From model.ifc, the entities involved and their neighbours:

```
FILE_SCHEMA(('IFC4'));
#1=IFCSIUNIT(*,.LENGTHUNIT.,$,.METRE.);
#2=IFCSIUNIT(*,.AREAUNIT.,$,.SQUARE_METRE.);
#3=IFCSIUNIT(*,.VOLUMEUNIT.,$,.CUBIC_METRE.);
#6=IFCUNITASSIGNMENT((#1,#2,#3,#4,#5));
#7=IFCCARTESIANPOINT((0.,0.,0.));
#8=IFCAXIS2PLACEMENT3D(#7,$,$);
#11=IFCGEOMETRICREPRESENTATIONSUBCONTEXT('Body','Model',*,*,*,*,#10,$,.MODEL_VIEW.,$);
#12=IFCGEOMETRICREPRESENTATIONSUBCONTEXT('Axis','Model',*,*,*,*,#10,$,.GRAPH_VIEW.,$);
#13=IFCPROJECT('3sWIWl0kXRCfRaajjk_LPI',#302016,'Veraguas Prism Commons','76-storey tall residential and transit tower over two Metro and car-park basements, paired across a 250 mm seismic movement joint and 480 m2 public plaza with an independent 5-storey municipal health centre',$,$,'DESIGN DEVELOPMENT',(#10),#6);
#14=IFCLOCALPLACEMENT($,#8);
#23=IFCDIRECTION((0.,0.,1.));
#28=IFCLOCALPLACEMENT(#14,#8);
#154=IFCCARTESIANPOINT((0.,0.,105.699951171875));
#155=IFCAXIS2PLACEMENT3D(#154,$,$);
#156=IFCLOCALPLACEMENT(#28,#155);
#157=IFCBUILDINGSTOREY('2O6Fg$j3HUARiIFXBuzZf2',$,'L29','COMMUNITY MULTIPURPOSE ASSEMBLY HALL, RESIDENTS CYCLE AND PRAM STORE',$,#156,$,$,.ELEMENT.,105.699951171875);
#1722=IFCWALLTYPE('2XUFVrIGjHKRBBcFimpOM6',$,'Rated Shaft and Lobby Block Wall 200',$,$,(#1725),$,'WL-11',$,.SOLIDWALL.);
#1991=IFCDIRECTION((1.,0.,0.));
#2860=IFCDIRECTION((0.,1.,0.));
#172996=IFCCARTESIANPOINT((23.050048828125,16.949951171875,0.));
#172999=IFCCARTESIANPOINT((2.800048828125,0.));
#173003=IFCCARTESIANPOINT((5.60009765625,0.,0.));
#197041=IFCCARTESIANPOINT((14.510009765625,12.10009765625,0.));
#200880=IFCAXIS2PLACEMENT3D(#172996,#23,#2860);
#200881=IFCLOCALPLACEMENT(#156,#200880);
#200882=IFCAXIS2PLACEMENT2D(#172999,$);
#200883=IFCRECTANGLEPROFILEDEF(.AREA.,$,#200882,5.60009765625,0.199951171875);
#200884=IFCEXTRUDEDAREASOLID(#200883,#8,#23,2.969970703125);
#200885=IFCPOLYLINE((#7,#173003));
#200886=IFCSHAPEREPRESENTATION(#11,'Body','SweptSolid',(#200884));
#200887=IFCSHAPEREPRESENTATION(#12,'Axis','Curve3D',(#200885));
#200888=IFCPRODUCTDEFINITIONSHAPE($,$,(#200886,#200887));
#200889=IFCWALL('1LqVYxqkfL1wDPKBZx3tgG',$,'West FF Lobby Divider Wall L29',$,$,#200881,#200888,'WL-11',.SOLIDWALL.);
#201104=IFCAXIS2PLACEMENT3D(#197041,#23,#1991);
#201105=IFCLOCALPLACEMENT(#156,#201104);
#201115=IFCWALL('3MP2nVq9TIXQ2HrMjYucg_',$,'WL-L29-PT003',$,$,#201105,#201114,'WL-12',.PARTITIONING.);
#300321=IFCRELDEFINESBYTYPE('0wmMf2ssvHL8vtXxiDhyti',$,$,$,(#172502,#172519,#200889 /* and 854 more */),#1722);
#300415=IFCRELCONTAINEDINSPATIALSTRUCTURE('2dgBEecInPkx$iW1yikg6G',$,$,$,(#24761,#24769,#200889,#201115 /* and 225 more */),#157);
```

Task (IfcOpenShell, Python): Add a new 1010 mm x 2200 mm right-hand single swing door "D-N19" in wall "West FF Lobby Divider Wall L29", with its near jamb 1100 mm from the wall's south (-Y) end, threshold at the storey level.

```python
import numpy as np
import ifcopenshell
import ifcopenshell.api.feature
import ifcopenshell.api.geometry
import ifcopenshell.api.root
import ifcopenshell.api.spatial
import ifcopenshell.geom
import ifcopenshell.util.element
import ifcopenshell.util.placement
import ifcopenshell.util.representation
import ifcopenshell.util.shape
import ifcopenshell.util.unit

model = ifcopenshell.open("model.ifc")
unit_scale = ifcopenshell.util.unit.calculate_unit_scale(model)
settings = ifcopenshell.geom.settings()


def volume(element):
    """Net volume in cubic metres, openings subtracted."""
    shape = ifcopenshell.geom.create_shape(settings, element)
    return ifcopenshell.util.shape.get_volume(shape.geometry)


wall = model.by_guid("1LqVYxqkfL1wDPKBZx3tgG")
storey = ifcopenshell.util.element.get_container(wall, ifc_class="IfcBuildingStorey")
context = ifcopenshell.util.representation.get_context(model, "Model", "Body", "MODEL_VIEW")
before = volume(wall)

width, height, from_end, sill = 1.01, 2.2, 1.1, 0.0  # metres

# The wall runs along its own X axis, and the end named is its -X end.
wall_shape = ifcopenshell.geom.create_shape(settings, wall)
x, y, z = ifcopenshell.util.shape.get_vertices(wall_shape.geometry).T
start = x.min() + from_end
face, thickness = float(y.min()), float(y.max() - y.min())
wall_matrix = ifcopenshell.util.placement.get_local_placement(wall.ObjectPlacement)
level = ifcopenshell.util.placement.get_local_placement(storey.ObjectPlacement)[2, 3]


def in_wall(x, y):
    """Placement at x, y metres in the wall's axes, at sill height."""
    matrix = wall_matrix.copy()
    matrix[:, 3] = wall_matrix @ np.array([x / unit_scale, y / unit_scale, 0.0, 1.0])
    matrix[2, 3] = level + sill / unit_scale
    return matrix


# Opening: a box that overshoots both wall faces by 50 mm.
opening = ifcopenshell.api.root.create_entity(model, ifc_class="IfcOpeningElement", predefined_type="OPENING")
box = ifcopenshell.api.geometry.add_wall_representation(
    model, context=context, length=width, height=height, thickness=thickness + 0.1
)
ifcopenshell.api.geometry.assign_representation(model, product=opening, representation=box)
ifcopenshell.api.geometry.edit_object_placement(model, product=opening, matrix=in_wall(start, face - 0.05), is_si=False)
ifcopenshell.api.feature.add_feature(model, feature=opening, element=wall)

door = ifcopenshell.api.root.create_entity(model, ifc_class="IfcDoor", name="D-N19", predefined_type="DOOR")
door.OverallWidth, door.OverallHeight = width / unit_scale, height / unit_scale
door.OperationType = "SINGLE_SWING_RIGHT"
body = ifcopenshell.api.geometry.add_door_representation(
    model,
    context=context,
    overall_width=door.OverallWidth,
    overall_height=door.OverallHeight,
    operation_type="SINGLE_SWING_RIGHT",
    lining_properties={"LiningDepth": thickness / unit_scale, "ThresholdDepth": thickness / unit_scale},
)
ifcopenshell.api.geometry.assign_representation(model, product=door, representation=body)
ifcopenshell.api.spatial.assign_container(model, products=[door], relating_structure=storey)
ifcopenshell.api.feature.add_filling(model, opening=opening, element=door)

# The lining spans the wall, so the door starts at the wall face.
ifcopenshell.api.geometry.edit_object_placement(model, product=door, matrix=in_wall(start, face), is_si=False)

after = volume(wall)

print(f"wall volume {before:.3f} -> {after:.3f} m3")

model.write("model_v2.ifc")
```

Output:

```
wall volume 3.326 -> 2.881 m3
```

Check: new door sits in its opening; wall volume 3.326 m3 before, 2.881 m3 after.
